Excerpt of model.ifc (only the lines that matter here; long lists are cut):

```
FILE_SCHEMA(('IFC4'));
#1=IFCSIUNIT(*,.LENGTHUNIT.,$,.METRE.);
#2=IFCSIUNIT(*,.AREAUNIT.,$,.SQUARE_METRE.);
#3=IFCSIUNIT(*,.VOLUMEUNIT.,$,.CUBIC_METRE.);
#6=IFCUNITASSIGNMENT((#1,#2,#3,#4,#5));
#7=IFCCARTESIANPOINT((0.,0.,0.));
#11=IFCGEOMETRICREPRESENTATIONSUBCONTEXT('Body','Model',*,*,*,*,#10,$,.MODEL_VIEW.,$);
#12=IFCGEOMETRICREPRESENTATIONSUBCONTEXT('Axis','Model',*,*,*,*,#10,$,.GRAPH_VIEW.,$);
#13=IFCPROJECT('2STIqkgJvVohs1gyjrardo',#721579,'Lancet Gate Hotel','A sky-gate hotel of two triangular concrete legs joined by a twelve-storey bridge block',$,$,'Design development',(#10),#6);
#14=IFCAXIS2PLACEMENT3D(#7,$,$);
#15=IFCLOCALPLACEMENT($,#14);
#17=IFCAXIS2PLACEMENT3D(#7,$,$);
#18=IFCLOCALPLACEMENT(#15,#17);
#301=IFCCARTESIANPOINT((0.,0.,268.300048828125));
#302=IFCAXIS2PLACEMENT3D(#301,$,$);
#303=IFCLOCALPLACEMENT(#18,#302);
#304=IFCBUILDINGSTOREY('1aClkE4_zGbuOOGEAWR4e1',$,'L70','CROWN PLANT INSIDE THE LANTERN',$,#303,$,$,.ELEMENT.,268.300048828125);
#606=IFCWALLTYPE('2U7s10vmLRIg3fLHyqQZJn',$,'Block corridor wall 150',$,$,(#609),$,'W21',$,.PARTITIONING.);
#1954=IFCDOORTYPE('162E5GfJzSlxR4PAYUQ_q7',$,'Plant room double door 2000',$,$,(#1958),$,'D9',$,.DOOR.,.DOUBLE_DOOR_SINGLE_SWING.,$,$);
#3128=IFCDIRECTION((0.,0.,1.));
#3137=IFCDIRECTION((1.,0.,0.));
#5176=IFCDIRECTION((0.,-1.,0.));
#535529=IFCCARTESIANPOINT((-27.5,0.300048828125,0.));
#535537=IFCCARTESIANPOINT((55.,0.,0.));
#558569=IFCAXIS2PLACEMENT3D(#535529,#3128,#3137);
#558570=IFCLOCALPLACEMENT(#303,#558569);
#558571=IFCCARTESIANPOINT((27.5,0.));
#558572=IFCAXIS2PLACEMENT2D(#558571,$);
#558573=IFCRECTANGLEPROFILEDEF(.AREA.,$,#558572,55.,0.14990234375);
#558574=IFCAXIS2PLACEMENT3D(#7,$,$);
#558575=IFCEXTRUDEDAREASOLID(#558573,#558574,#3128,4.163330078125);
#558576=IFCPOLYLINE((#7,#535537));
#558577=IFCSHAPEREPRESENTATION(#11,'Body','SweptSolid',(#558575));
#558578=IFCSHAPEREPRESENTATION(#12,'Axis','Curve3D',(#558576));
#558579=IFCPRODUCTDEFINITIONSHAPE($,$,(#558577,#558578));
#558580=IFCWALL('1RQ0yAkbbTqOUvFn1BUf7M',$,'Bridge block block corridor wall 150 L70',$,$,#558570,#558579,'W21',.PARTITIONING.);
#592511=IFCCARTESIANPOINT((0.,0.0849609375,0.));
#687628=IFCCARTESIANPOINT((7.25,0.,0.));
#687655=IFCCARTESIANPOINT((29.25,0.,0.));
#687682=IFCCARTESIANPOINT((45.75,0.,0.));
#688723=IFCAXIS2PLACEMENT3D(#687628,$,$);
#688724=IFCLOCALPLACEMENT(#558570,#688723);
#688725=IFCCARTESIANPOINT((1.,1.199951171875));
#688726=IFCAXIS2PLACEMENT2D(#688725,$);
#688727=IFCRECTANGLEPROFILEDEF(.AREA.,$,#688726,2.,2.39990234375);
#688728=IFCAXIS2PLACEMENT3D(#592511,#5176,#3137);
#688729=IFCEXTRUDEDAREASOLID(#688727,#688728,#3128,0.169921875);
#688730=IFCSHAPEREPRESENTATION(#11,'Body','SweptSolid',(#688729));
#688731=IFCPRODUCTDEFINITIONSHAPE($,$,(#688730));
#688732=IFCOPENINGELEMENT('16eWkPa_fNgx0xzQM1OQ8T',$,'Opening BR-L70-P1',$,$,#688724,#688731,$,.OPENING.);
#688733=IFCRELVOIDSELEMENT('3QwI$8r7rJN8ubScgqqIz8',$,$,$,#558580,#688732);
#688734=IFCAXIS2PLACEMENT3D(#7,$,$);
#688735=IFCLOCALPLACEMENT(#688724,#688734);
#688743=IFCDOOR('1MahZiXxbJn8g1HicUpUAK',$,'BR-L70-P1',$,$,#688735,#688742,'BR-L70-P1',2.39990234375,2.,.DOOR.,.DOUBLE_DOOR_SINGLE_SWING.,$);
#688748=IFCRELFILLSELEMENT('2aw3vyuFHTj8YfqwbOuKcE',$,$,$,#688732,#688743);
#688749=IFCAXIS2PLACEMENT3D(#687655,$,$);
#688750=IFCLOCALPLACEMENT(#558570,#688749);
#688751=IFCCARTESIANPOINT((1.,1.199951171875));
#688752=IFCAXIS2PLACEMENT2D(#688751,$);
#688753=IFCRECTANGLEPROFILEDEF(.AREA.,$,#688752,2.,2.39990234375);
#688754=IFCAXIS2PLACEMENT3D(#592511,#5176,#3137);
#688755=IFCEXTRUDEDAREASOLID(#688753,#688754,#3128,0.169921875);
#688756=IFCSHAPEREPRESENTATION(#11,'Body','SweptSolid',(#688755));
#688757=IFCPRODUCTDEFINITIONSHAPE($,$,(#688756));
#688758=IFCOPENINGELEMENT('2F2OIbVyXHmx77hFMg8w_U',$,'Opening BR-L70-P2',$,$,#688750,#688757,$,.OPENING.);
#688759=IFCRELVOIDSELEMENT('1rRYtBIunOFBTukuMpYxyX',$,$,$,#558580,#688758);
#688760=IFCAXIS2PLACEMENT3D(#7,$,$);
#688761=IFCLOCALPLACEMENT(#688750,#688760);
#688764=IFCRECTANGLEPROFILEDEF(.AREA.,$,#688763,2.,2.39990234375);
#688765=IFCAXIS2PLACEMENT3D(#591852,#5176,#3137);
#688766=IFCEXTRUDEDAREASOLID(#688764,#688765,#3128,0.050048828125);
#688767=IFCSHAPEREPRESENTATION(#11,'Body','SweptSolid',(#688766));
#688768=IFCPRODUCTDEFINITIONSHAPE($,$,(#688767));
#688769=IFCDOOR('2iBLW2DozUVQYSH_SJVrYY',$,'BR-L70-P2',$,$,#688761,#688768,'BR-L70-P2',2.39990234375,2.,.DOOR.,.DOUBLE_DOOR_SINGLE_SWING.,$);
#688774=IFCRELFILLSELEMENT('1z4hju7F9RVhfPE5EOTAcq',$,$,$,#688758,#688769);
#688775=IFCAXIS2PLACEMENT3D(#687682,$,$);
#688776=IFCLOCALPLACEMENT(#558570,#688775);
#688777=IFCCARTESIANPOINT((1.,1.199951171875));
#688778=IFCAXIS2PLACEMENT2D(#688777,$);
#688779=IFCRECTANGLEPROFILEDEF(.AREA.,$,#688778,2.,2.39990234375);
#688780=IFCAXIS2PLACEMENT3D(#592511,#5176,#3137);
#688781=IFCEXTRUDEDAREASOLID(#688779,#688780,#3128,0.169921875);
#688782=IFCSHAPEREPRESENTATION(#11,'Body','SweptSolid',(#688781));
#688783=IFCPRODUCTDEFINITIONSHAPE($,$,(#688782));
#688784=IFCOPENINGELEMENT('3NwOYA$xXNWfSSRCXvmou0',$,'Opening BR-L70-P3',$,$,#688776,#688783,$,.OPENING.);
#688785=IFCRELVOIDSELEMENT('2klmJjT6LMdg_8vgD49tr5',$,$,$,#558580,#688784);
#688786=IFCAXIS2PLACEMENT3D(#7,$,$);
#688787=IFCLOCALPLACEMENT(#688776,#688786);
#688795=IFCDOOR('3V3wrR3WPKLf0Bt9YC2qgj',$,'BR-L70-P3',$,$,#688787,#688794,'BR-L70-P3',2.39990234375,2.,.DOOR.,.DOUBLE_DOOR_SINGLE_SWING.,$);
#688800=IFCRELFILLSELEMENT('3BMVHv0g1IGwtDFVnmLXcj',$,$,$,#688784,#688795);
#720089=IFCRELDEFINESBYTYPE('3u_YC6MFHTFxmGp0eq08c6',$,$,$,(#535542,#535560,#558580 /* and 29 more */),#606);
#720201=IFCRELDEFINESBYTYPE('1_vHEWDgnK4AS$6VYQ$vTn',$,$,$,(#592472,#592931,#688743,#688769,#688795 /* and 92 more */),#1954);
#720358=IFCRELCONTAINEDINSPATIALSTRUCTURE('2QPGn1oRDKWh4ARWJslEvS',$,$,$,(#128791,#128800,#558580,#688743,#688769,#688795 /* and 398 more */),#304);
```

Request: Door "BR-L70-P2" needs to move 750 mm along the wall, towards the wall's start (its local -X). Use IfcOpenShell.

```python
import ifcopenshell
import ifcopenshell.api.geometry
import ifcopenshell.util.placement
import ifcopenshell.util.unit

model = ifcopenshell.open("model.ifc")
unit_scale = ifcopenshell.util.unit.calculate_unit_scale(model)

door = model.by_guid("2iBLW2DozUVQYSH_SJVrYY")
opening = door.FillsVoids[0].RelatingOpeningElement
wall = opening.VoidsElements[0].RelatingBuildingElement

wall_matrix = ifcopenshell.util.placement.get_local_placement(wall.ObjectPlacement)
shift = wall_matrix[:3, 0] * -0.75 / unit_scale
before = ifcopenshell.util.placement.get_local_placement(door.ObjectPlacement)[:3, 3].copy()

# The door is placed relative to its opening, so it follows when the opening moves.
matrix = ifcopenshell.util.placement.get_local_placement(opening.ObjectPlacement)
matrix[:3, 3] += shift
ifcopenshell.api.geometry.edit_object_placement(
    model, product=opening, matrix=matrix, is_si=False, should_transform_children=True
)

after = ifcopenshell.util.placement.get_local_placement(door.ObjectPlacement)[:3, 3]
print("door moved by", (after - before).round(3) + 0.0)

model.write("model_updated.ifc")
```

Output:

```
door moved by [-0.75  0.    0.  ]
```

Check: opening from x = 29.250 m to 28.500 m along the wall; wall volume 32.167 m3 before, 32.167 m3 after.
